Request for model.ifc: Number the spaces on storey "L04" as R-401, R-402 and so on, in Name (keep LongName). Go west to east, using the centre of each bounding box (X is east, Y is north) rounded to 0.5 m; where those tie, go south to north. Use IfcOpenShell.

First a look at what the model holds.

```python
import ifcopenshell
import ifcopenshell.util.element
import ifcopenshell.util.placement

model = ifcopenshell.open("model.ifc")
print(model.schema)
storey = next(s for s in model.by_type("IfcBuildingStorey") if s.Name == "L04")
spaces = [e for e in ifcopenshell.util.element.get_decomposition(storey) if e.is_a("IfcSpace")]
for e in sorted(spaces, key=lambda e: e.id()):
    origin = ifcopenshell.util.placement.get_local_placement(e.ObjectPlacement)[:3, 3]
    print(e.id(), e.Name, e.LongName, origin.round(2) + 0.0, sep=" | ")
```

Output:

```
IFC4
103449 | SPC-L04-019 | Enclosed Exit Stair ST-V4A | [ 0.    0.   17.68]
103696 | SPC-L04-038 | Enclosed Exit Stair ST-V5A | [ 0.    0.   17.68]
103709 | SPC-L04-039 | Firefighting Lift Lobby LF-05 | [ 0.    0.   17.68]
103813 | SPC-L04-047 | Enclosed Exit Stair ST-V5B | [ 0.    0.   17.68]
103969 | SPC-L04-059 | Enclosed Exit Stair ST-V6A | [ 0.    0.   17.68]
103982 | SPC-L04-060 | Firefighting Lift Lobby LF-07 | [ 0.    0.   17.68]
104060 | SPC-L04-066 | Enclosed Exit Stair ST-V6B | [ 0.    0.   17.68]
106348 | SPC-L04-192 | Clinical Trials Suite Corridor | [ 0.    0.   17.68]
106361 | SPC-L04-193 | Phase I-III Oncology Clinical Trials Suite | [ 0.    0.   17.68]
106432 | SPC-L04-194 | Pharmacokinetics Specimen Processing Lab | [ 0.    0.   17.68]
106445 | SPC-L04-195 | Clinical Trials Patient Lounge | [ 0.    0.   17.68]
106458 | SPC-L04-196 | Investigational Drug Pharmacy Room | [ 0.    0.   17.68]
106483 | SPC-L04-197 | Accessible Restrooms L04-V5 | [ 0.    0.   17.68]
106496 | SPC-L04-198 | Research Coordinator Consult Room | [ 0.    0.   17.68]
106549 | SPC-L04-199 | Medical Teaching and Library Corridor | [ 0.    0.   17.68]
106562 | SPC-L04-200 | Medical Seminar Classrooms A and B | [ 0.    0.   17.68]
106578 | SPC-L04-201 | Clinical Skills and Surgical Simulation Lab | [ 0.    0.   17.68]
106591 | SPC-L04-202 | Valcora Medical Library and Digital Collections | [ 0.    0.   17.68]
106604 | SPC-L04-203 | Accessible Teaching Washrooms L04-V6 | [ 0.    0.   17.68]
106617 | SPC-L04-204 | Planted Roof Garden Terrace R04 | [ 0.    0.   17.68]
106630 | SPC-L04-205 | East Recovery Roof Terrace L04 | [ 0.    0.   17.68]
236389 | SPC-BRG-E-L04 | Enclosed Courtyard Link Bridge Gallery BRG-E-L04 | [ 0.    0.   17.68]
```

```python
import ifcopenshell
import ifcopenshell.geom
import ifcopenshell.util.element
import ifcopenshell.util.shape

model = ifcopenshell.open("model.ifc")
settings = ifcopenshell.geom.settings()
settings.set("use-world-coords", True)


def centre(element):
    shape = ifcopenshell.geom.create_shape(settings, element)
    return ifcopenshell.util.shape.get_bbox_centroid(shape.geometry)


storey = next(s for s in model.by_type("IfcBuildingStorey") if s.Name == "L04")
spaces = [e for e in ifcopenshell.util.element.get_decomposition(storey) if e.is_a("IfcSpace")]

# Insertion points can sit at a corner or the storey origin, so sort by the geometry (in metres).
centres = {e: centre(e) for e in spaces}
spaces.sort(key=lambda e: (round(centres[e][0] / 0.5), centres[e][1]))

for i, e in enumerate(spaces, start=1):
    number = f"R-4{i:02d}"
    e.Name = number
    print(e.id(), number)

model.write("model_v2.ifc")
```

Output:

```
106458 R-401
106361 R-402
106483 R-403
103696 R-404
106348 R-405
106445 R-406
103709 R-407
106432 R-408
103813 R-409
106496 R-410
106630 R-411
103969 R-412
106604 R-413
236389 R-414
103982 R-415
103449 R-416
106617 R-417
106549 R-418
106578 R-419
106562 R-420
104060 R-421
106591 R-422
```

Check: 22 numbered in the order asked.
